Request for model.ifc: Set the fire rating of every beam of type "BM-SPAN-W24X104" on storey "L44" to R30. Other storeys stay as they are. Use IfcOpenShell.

First a look at what the model holds.

```python
import ifcopenshell
import ifcopenshell.util.element

model = ifcopenshell.open("model.ifc")
print(model.schema)
storey = next(s for s in model.by_type("IfcBuildingStorey") if s.Name == "L44")
beams = [e for e in ifcopenshell.util.element.get_decomposition(storey) if e.is_a("IfcBeam")]
seen = {}
for e in beams:
    element_type = ifcopenshell.util.element.get_type(e)
    key = (element_type.Name if element_type != e and element_type else None, ifcopenshell.util.element.get_pset(e, "Pset_BeamCommon", "FireRating"))
    seen[key] = seen.get(key, 0) + 1
for (name, value), count in sorted(seen.items(), key=str):
    print(count, "x", name, "|", value)
```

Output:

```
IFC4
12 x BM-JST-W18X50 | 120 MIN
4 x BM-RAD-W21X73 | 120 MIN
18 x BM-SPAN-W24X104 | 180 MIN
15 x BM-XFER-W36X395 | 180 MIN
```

```python
import ifcopenshell
import ifcopenshell.api.pset
import ifcopenshell.util.element

model = ifcopenshell.open("model.ifc")

storey = next(s for s in model.by_type("IfcBuildingStorey") if s.Name == "L44")
beams = [e for e in ifcopenshell.util.element.get_decomposition(storey) if e.is_a("IfcBeam")]

count = 0
for e in beams:
    element_type = ifcopenshell.util.element.get_type(e)
    if element_type in (None, e) or element_type.Name != "BM-SPAN-W24X104":
        continue
    found = ifcopenshell.util.element.get_pset(e, "Pset_BeamCommon", should_inherit=False)
    if found:
        pset = model.by_id(found["id"])
        if len(ifcopenshell.util.element.get_elements_by_pset(pset)) > 1:
            pset = ifcopenshell.api.pset.unshare_pset(model, products=[e], pset=pset)[0]
    else:
        pset = ifcopenshell.api.pset.add_pset(model, product=e, name="Pset_BeamCommon")
    ifcopenshell.api.pset.edit_pset(model, pset=pset, properties={"FireRating": "R30"})
    count += 1

print(count, "beams updated")

model.write("model_rev.ifc")
```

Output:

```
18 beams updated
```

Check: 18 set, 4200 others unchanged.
